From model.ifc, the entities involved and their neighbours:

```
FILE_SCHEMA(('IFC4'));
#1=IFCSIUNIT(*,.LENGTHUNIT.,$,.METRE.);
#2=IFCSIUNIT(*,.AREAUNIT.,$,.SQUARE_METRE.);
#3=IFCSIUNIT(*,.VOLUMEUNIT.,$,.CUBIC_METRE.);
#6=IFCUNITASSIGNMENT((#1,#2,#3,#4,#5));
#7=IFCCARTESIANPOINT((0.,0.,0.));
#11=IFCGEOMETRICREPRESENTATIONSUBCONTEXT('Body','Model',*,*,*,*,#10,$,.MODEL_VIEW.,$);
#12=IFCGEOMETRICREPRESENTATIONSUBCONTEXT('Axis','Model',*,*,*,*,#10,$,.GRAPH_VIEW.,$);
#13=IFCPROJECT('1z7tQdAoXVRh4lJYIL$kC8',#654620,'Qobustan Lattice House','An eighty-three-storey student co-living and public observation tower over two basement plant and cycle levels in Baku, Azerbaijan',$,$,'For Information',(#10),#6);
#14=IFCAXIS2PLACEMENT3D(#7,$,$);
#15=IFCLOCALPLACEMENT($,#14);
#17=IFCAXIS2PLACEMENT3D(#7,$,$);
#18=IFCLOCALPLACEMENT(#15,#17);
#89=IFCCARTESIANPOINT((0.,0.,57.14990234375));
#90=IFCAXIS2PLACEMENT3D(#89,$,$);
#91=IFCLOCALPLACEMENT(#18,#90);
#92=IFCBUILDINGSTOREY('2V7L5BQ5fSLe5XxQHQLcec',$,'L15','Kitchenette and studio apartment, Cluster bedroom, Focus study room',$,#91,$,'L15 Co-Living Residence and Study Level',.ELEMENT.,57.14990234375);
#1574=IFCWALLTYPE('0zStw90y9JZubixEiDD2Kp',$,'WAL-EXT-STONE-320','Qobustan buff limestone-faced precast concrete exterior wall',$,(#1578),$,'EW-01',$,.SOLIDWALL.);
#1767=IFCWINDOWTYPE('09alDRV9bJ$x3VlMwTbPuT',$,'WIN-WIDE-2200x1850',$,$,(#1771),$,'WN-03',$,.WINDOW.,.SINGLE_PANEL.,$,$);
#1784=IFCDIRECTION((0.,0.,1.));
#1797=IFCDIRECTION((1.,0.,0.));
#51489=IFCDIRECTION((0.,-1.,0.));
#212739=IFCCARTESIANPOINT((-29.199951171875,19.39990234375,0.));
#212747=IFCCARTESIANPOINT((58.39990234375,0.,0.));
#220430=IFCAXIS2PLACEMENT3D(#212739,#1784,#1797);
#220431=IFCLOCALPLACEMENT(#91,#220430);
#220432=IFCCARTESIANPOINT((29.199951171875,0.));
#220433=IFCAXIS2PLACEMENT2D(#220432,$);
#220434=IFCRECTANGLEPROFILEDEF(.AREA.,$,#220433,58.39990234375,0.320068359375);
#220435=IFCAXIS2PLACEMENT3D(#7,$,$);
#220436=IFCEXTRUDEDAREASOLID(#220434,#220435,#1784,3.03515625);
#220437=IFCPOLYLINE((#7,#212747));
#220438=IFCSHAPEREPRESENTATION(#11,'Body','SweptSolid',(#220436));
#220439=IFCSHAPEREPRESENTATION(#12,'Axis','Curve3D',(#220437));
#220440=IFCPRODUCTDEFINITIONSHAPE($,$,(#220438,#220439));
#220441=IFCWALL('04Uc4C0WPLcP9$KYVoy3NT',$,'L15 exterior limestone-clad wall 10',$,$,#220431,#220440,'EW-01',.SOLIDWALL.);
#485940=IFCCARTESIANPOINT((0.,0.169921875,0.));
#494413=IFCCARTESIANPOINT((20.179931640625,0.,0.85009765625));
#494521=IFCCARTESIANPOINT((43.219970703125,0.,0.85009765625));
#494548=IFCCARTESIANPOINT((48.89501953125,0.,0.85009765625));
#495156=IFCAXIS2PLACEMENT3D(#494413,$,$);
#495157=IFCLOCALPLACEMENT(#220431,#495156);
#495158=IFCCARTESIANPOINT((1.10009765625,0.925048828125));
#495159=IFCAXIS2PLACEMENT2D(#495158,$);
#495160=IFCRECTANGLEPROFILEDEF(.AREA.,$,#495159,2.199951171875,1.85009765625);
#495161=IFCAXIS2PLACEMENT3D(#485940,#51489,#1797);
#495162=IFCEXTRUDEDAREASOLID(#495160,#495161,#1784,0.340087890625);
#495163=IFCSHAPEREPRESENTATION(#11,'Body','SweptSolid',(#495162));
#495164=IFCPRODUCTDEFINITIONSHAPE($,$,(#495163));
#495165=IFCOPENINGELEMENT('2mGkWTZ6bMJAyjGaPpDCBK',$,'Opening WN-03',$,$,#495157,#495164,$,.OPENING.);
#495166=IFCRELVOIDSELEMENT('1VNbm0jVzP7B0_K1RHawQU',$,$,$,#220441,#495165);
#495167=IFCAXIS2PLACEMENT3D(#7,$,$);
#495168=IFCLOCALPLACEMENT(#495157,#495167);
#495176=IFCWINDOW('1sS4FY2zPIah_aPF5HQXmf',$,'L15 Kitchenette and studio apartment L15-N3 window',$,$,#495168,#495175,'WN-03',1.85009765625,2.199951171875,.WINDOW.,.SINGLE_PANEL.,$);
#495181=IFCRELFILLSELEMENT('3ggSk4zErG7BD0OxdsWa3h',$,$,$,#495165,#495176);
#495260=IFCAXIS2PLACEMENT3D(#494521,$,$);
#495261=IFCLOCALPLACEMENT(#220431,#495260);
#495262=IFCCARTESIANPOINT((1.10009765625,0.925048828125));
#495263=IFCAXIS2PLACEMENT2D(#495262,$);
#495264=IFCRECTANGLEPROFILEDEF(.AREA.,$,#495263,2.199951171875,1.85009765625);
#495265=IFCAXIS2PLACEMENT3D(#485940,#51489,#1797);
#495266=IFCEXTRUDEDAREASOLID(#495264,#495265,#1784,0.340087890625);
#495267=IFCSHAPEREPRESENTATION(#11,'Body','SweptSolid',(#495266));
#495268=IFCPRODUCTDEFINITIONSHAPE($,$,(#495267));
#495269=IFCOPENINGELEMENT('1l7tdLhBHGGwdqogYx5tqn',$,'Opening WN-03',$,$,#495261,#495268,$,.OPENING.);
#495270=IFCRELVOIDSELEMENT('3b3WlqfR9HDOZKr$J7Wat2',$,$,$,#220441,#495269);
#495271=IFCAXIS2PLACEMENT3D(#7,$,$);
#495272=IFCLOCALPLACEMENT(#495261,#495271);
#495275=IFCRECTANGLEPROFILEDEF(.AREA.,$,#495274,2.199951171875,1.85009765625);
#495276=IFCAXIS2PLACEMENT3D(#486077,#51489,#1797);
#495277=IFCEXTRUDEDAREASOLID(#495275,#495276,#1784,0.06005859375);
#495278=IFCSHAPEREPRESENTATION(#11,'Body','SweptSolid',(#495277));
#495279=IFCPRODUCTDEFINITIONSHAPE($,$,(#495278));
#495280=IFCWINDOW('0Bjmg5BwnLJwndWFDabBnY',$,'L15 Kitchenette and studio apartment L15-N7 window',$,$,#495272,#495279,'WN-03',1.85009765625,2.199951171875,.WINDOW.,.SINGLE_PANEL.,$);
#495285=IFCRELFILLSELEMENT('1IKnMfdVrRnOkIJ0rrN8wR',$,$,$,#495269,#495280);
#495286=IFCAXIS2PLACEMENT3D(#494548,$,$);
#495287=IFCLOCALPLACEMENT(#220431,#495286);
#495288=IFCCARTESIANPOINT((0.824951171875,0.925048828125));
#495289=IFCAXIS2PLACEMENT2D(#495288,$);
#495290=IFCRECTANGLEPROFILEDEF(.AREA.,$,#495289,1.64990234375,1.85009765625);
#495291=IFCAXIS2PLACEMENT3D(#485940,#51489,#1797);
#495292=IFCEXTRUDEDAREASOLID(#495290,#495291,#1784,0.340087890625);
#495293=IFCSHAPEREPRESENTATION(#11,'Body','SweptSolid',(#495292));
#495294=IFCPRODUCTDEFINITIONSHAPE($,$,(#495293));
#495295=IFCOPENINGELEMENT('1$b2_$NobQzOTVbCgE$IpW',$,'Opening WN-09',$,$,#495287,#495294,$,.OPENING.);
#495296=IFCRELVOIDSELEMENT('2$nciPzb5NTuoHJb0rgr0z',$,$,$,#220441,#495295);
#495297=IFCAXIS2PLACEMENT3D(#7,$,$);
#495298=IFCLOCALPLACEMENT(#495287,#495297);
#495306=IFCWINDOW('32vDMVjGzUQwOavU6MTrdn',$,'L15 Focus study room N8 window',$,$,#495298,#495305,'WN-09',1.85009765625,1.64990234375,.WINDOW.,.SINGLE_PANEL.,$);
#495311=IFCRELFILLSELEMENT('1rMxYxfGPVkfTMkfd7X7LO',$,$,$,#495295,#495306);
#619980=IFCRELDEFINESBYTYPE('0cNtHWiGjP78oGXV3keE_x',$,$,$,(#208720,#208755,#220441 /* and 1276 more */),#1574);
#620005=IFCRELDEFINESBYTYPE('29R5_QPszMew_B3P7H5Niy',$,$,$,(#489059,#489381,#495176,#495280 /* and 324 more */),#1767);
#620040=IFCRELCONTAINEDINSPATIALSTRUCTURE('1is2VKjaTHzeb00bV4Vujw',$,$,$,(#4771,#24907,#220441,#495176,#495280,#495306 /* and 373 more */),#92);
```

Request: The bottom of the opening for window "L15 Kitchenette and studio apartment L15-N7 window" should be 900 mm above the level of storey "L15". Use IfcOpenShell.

```python
import numpy as np
import ifcopenshell
import ifcopenshell.api.geometry
import ifcopenshell.geom
import ifcopenshell.util.element
import ifcopenshell.util.placement
import ifcopenshell.util.shape
import ifcopenshell.util.unit

model = ifcopenshell.open("model.ifc")
unit_scale = ifcopenshell.util.unit.calculate_unit_scale(model)

window = model.by_guid("0Bjmg5BwnLJwndWFDabBnY")
opening = window.FillsVoids[0].RelatingOpeningElement
storey = ifcopenshell.util.element.get_container(window, ifc_class="IfcBuildingStorey")
level = ifcopenshell.util.placement.get_local_placement(storey.ObjectPlacement)[2, 3]

# The opening's origin need not be at the sill, so measure its lowest point.
shape = ifcopenshell.geom.create_shape(ifcopenshell.geom.settings(), opening)
bottom = ifcopenshell.util.shape.get_shape_bottom_elevation(shape, shape.geometry) / unit_scale
dz = level + 0.9 / unit_scale - bottom

shift = np.array([0.0, 0.0, dz])
# The window is placed relative to its opening, so it follows when the opening moves.
matrix = ifcopenshell.util.placement.get_local_placement(opening.ObjectPlacement)
matrix[:3, 3] += shift
ifcopenshell.api.geometry.edit_object_placement(
    model, product=opening, matrix=matrix, is_si=False, should_transform_children=True
)

print(f"moved by {dz * unit_scale:+.3f} m")

model.write("model_edited.ifc")
```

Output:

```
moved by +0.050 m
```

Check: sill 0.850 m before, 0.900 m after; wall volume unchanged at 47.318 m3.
